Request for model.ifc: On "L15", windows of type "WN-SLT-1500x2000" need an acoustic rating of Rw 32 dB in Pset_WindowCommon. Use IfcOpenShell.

First a look at what the model holds.

```python
import ifcopenshell
import ifcopenshell.util.element

model = ifcopenshell.open("model.ifc")
print(model.schema)
storey = next(s for s in model.by_type("IfcBuildingStorey") if s.Name == "L15")
windows = [e for e in ifcopenshell.util.element.get_decomposition(storey) if e.is_a("IfcWindow")]
seen = {}
for e in windows:
    element_type = ifcopenshell.util.element.get_type(e)
    key = (element_type.Name if element_type != e and element_type else None, ifcopenshell.util.element.get_pset(e, "Pset_WindowCommon", "AcousticRating"))
    seen[key] = seen.get(key, 0) + 1
for (name, value), count in sorted(seen.items(), key=str):
    print(count, "x", name, "|", value)
```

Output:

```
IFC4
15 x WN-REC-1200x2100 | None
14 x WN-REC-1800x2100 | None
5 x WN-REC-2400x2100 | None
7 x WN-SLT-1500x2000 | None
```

```python
import ifcopenshell
import ifcopenshell.api.pset
import ifcopenshell.util.element

model = ifcopenshell.open("model.ifc")

storey = next(s for s in model.by_type("IfcBuildingStorey") if s.Name == "L15")
windows = [e for e in ifcopenshell.util.element.get_decomposition(storey) if e.is_a("IfcWindow")]

count = 0
for e in windows:
    element_type = ifcopenshell.util.element.get_type(e)
    if element_type in (None, e) or element_type.Name != "WN-SLT-1500x2000":
        continue
    found = ifcopenshell.util.element.get_pset(e, "Pset_WindowCommon", should_inherit=False)
    if found:
        pset = model.by_id(found["id"])
        if len(ifcopenshell.util.element.get_elements_by_pset(pset)) > 1:
            pset = ifcopenshell.api.pset.unshare_pset(model, products=[e], pset=pset)[0]
    else:
        pset = ifcopenshell.api.pset.add_pset(model, product=e, name="Pset_WindowCommon")
    ifcopenshell.api.pset.edit_pset(model, pset=pset, properties={"AcousticRating": "Rw 32 dB"})
    count += 1

print(count, "windows updated")

model.write("model_v2.ifc")
```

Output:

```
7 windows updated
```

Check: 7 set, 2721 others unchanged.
